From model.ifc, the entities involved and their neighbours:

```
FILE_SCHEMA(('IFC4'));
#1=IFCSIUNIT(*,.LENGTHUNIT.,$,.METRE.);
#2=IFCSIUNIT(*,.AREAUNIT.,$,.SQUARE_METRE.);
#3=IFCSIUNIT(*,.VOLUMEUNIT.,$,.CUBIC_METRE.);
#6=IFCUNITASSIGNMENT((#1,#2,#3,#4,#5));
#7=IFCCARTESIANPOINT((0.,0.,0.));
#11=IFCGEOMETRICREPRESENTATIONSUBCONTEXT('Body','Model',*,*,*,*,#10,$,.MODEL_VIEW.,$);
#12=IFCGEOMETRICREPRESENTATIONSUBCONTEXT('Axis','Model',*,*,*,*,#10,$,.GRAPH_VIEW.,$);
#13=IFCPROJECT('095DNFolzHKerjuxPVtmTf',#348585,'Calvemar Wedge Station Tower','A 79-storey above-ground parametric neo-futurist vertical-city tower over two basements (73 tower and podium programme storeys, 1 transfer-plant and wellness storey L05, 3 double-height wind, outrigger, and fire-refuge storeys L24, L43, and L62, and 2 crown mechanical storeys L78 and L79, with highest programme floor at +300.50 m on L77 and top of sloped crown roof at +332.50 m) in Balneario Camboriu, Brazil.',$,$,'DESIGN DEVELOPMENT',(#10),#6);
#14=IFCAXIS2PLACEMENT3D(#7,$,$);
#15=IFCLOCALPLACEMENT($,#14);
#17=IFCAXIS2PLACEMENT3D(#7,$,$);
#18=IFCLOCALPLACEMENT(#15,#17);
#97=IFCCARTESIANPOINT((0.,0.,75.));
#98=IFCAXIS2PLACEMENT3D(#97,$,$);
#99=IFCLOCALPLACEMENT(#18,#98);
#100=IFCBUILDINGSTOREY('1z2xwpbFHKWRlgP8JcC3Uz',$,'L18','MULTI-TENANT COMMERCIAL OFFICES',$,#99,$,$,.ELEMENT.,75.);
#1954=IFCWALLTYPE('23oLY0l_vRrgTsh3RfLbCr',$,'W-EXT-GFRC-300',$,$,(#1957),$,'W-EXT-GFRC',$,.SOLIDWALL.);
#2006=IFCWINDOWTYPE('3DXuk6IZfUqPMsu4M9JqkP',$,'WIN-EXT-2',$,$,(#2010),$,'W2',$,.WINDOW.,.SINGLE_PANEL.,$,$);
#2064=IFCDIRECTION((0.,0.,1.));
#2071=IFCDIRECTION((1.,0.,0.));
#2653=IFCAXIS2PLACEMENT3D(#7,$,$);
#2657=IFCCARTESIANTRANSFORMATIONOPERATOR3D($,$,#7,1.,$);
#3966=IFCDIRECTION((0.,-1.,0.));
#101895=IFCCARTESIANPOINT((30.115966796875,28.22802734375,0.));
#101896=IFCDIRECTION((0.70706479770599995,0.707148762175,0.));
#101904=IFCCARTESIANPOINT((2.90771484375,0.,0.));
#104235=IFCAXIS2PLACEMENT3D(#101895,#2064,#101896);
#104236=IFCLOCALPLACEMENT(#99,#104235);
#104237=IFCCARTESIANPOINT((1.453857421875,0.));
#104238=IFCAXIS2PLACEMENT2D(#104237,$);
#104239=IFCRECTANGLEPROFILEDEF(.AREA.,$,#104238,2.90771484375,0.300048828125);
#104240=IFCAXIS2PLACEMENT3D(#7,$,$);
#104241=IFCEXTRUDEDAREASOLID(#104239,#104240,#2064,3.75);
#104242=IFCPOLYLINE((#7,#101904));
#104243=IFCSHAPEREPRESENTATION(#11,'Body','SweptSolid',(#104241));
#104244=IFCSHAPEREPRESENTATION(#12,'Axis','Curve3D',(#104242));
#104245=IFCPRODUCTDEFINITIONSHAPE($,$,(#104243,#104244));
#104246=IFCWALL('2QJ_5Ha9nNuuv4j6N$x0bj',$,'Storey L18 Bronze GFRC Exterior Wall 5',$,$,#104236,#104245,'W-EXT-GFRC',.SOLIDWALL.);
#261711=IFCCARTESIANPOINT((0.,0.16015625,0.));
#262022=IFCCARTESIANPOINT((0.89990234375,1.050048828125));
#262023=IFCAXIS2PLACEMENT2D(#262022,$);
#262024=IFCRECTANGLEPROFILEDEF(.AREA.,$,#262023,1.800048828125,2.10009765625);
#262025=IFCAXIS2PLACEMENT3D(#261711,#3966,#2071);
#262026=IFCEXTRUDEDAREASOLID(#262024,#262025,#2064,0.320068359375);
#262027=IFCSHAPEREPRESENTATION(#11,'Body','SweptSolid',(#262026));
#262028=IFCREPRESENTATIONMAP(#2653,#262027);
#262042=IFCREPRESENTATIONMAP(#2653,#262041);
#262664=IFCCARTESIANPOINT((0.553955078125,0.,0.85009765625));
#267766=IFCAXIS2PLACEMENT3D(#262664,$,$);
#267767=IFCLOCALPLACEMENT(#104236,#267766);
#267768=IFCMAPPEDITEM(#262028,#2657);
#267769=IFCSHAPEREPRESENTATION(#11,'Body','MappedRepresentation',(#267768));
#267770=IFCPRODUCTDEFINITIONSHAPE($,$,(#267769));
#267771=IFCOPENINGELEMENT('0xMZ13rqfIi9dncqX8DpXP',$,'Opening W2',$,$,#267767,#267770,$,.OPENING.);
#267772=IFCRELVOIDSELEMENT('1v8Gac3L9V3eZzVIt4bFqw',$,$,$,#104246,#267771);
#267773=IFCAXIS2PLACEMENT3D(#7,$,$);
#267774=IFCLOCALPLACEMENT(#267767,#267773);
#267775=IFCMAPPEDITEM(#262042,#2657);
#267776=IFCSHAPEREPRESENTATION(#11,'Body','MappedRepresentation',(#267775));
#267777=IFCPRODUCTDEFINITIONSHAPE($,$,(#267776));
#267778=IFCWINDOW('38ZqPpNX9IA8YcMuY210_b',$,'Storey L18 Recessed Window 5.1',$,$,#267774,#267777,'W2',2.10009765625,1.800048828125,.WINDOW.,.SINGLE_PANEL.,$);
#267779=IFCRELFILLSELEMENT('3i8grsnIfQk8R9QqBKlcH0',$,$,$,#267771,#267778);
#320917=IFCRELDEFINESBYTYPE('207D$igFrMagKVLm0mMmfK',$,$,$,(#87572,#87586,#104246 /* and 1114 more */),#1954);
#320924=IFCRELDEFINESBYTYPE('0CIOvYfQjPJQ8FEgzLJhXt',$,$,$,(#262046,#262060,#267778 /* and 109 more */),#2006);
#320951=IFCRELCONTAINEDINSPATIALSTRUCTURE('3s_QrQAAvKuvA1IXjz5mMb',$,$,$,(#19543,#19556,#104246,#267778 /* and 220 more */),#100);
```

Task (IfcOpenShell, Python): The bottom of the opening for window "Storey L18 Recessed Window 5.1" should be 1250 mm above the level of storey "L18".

```python
import numpy as np
import ifcopenshell
import ifcopenshell.api.geometry
import ifcopenshell.geom
import ifcopenshell.util.element
import ifcopenshell.util.placement
import ifcopenshell.util.shape
import ifcopenshell.util.unit

model = ifcopenshell.open("model.ifc")
unit_scale = ifcopenshell.util.unit.calculate_unit_scale(model)

window = model.by_guid("38ZqPpNX9IA8YcMuY210_b")
opening = window.FillsVoids[0].RelatingOpeningElement
storey = ifcopenshell.util.element.get_container(window, ifc_class="IfcBuildingStorey")
level = ifcopenshell.util.placement.get_local_placement(storey.ObjectPlacement)[2, 3]

# The opening's origin need not be at the sill, so measure its lowest point.
shape = ifcopenshell.geom.create_shape(ifcopenshell.geom.settings(), opening)
bottom = ifcopenshell.util.shape.get_shape_bottom_elevation(shape, shape.geometry) / unit_scale
dz = level + 1.25 / unit_scale - bottom

shift = np.array([0.0, 0.0, dz])
# The window is placed relative to its opening, so it follows when the opening moves.
matrix = ifcopenshell.util.placement.get_local_placement(opening.ObjectPlacement)
matrix[:3, 3] += shift
ifcopenshell.api.geometry.edit_object_placement(
    model, product=opening, matrix=matrix, is_si=False, should_transform_children=True
)

print(f"moved by {dz * unit_scale:+.3f} m")

model.write("model-out.ifc")
```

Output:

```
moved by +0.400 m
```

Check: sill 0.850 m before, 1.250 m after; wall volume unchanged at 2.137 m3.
